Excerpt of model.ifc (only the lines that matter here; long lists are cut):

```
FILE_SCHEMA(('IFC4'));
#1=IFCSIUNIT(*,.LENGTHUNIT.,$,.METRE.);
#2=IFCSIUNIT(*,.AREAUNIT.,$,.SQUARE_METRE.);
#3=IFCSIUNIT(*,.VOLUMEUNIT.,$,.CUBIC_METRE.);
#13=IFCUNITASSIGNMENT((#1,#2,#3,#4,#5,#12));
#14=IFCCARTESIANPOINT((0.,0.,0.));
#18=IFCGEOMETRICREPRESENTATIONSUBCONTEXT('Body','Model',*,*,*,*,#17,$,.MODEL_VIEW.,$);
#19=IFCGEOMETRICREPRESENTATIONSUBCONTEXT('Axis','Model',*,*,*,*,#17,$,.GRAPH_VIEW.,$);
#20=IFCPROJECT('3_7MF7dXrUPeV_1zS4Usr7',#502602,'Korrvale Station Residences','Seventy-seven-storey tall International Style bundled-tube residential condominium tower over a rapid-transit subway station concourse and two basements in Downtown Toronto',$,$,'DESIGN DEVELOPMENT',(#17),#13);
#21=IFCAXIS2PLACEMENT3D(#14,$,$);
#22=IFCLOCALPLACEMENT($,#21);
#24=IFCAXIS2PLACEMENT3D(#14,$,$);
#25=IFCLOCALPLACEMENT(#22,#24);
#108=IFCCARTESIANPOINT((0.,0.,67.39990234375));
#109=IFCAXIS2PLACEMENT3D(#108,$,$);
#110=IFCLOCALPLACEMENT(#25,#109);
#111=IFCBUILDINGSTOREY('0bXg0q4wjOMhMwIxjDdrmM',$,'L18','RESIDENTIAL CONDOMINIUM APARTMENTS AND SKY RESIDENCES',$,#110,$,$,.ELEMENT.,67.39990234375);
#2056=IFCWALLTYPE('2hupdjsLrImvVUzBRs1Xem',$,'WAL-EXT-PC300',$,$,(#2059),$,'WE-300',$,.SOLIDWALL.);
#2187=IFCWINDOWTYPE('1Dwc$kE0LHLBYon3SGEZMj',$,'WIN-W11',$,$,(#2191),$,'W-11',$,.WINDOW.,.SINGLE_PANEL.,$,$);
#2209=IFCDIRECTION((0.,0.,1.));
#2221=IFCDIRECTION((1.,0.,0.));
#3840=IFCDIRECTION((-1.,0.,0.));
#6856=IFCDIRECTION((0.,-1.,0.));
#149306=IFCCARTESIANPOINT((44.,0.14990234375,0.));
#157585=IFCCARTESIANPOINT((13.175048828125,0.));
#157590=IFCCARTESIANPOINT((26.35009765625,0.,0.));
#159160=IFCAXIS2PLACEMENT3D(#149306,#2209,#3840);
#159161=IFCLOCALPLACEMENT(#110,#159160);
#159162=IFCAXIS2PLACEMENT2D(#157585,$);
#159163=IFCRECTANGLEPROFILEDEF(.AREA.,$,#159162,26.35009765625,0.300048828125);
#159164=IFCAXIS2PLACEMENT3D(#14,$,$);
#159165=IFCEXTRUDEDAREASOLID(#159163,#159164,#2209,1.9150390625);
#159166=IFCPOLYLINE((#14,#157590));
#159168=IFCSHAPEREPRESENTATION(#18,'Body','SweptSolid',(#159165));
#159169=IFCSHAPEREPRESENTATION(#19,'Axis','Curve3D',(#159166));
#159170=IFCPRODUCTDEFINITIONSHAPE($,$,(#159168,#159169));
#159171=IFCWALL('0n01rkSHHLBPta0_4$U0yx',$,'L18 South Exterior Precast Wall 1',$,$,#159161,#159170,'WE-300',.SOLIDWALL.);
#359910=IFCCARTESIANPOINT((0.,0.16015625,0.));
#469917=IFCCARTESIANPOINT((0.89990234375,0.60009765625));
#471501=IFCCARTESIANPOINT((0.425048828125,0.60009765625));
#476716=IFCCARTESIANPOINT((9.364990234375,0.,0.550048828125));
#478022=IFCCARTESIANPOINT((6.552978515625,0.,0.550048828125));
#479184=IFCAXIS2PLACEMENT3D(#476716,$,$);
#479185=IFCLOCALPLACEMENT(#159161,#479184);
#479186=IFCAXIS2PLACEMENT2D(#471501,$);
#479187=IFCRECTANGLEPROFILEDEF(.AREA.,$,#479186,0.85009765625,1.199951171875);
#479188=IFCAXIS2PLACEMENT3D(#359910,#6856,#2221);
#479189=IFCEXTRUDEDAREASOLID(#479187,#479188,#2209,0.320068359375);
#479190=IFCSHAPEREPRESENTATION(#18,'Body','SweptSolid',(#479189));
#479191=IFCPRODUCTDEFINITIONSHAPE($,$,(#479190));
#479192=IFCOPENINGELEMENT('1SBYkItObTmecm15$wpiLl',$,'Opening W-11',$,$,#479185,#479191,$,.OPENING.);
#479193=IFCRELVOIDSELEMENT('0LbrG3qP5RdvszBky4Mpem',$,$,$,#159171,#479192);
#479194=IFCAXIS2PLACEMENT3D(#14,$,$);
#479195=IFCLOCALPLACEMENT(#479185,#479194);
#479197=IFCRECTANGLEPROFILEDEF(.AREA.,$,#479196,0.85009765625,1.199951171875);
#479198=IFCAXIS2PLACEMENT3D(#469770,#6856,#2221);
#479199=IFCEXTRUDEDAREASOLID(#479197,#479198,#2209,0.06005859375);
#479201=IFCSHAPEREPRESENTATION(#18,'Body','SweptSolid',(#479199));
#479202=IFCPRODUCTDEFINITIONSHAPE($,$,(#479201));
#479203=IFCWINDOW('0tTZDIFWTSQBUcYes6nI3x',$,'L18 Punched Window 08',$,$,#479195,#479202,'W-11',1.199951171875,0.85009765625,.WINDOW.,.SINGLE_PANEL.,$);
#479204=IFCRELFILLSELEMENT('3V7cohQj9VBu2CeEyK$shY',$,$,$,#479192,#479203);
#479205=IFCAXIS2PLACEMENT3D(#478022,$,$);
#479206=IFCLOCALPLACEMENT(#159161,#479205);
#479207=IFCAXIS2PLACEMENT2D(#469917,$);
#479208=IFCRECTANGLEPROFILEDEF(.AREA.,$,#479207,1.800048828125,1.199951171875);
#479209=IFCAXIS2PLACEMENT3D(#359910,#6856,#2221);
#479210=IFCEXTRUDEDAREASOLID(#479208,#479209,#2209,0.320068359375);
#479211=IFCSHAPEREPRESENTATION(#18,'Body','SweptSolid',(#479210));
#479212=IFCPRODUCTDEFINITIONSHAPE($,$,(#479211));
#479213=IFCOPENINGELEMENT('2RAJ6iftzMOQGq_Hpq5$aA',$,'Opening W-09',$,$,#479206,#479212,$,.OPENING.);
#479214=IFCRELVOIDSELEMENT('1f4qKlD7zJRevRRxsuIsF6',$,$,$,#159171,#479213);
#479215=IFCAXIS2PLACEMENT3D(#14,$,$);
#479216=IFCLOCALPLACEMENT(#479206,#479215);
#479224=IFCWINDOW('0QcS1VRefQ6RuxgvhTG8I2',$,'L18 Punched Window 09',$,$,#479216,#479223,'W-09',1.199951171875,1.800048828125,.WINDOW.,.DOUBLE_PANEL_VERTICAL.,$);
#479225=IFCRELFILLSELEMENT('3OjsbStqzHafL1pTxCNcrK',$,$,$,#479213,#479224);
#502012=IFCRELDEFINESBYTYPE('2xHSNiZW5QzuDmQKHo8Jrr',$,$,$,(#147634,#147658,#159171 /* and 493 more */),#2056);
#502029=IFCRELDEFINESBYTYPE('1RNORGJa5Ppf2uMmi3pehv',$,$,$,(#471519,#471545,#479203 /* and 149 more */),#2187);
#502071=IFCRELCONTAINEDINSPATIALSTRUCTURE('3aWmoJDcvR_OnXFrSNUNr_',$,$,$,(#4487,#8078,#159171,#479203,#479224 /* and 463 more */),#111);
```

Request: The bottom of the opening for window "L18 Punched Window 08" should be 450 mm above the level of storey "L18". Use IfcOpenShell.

```python
import numpy as np
import ifcopenshell
import ifcopenshell.api.geometry
import ifcopenshell.geom
import ifcopenshell.util.element
import ifcopenshell.util.placement
import ifcopenshell.util.shape
import ifcopenshell.util.unit

model = ifcopenshell.open("model.ifc")
unit_scale = ifcopenshell.util.unit.calculate_unit_scale(model)

window = model.by_guid("0tTZDIFWTSQBUcYes6nI3x")
opening = window.FillsVoids[0].RelatingOpeningElement
storey = ifcopenshell.util.element.get_container(window, ifc_class="IfcBuildingStorey")
level = ifcopenshell.util.placement.get_local_placement(storey.ObjectPlacement)[2, 3]

# The opening's origin need not be at the sill, so measure its lowest point.
shape = ifcopenshell.geom.create_shape(ifcopenshell.geom.settings(), opening)
bottom = ifcopenshell.util.shape.get_shape_bottom_elevation(shape, shape.geometry) / unit_scale
dz = level + 0.45 / unit_scale - bottom

shift = np.array([0.0, 0.0, dz])
# The window is placed relative to its opening, so it follows when the opening moves.
matrix = ifcopenshell.util.placement.get_local_placement(opening.ObjectPlacement)
matrix[:3, 3] += shift
ifcopenshell.api.geometry.edit_object_placement(
    model, product=opening, matrix=matrix, is_si=False, should_transform_children=True
)

print(f"moved by {dz * unit_scale:+.3f} m")

model.write("model_updated.ifc")
```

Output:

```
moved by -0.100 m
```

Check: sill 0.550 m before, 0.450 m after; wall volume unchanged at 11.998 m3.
